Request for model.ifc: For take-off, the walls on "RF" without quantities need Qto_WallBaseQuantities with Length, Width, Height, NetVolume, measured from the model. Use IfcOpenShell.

First a look at what the model holds.

```python
import ifcopenshell
import ifcopenshell.util.element
import ifcopenshell.util.unit

model = ifcopenshell.open("model.ifc")
print(model.schema)
for unit_type in ("LENGTHUNIT", "AREAUNIT", "VOLUMEUNIT"):
    print(unit_type, ifcopenshell.util.unit.calculate_unit_scale(model, unit_type))
storey = next(s for s in model.by_type("IfcBuildingStorey") if s.Name == "RF")
walls = [e for e in ifcopenshell.util.element.get_decomposition(storey) if e.is_a("IfcWall")]
for e in sorted(walls, key=lambda e: e.id()):
    print(e.id(), e.is_a(), e.Name, list(ifcopenshell.util.element.get_psets(e, qtos_only=True)), sep=" | ")
```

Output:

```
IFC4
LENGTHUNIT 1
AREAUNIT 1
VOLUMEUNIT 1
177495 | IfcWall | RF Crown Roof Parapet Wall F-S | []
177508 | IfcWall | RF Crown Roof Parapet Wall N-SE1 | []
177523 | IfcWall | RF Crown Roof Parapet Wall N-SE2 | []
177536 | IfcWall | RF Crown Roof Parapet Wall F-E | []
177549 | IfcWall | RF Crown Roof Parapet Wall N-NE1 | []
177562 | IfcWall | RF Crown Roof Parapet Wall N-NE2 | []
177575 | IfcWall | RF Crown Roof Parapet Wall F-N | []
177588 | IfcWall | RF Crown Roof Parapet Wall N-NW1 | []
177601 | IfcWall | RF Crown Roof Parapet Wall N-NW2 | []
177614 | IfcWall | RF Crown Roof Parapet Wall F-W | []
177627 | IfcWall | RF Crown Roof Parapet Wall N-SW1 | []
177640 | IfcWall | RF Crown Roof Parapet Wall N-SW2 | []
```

```python
import ifcopenshell
import ifcopenshell.api.pset
import ifcopenshell.geom
import ifcopenshell.util.element
import ifcopenshell.util.shape
import ifcopenshell.util.unit

model = ifcopenshell.open("model.ifc")
unit_scale = ifcopenshell.util.unit.calculate_unit_scale(model)
volume_scale = ifcopenshell.util.unit.calculate_unit_scale(model, "VOLUMEUNIT")
settings = ifcopenshell.geom.settings()

storey = next(s for s in model.by_type("IfcBuildingStorey") if s.Name == "RF")
walls = [e for e in ifcopenshell.util.element.get_decomposition(storey) if e.is_a("IfcWall")]

for e in sorted(walls, key=lambda e: e.id()):
    if ifcopenshell.util.element.get_psets(e, qtos_only=True, should_inherit=False):
        continue
    # Geometry comes back in metres, in the element's own axes.
    shape = ifcopenshell.geom.create_shape(settings, e)
    values = {
        "Length": ifcopenshell.util.shape.get_x(shape.geometry) / unit_scale,
        "Width": ifcopenshell.util.shape.get_y(shape.geometry) / unit_scale,
        "Height": ifcopenshell.util.shape.get_z(shape.geometry) / unit_scale,
        "NetVolume": ifcopenshell.util.shape.get_volume(shape.geometry) / volume_scale,
    }
    qto = ifcopenshell.api.pset.add_qto(model, product=e, name="Qto_WallBaseQuantities")
    ifcopenshell.api.pset.edit_qto(model, qto=qto, properties=values)
    print(e.id(), {k: round(v, 3) for k, v in values.items()})

model.write("model_edited.ifc")
```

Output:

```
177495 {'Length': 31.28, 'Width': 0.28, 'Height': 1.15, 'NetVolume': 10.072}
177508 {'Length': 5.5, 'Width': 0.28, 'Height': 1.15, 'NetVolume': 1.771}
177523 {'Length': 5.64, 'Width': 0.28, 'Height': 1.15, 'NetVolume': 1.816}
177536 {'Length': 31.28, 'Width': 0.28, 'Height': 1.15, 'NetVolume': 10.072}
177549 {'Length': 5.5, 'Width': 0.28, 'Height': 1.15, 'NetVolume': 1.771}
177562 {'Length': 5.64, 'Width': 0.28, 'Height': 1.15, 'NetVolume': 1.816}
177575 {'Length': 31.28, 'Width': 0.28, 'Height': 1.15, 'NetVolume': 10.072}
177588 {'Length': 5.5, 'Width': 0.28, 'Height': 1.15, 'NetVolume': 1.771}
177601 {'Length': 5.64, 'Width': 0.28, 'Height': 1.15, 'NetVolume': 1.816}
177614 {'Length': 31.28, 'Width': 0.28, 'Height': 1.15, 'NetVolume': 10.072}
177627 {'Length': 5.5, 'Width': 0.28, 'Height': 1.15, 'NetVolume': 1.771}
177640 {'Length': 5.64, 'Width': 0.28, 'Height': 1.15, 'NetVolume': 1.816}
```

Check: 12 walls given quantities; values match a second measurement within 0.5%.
